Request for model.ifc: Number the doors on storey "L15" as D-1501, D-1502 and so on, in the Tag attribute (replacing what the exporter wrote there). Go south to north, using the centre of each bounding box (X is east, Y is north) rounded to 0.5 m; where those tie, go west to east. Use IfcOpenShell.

First a look at what the model holds.

```python
import ifcopenshell
import ifcopenshell.util.element
import ifcopenshell.util.placement

model = ifcopenshell.open("model.ifc")
print(model.schema)
storey = next(s for s in model.by_type("IfcBuildingStorey") if s.Name == "L15")
doors = [e for e in ifcopenshell.util.element.get_decomposition(storey) if e.is_a("IfcDoor")]
for e in sorted(doors, key=lambda e: e.id()):
    origin = ifcopenshell.util.placement.get_local_placement(e.ObjectPlacement)[:3, 3]
    print(e.id(), e.Tag, e.Name, origin.round(2) + 0.0, sep=" | ")
```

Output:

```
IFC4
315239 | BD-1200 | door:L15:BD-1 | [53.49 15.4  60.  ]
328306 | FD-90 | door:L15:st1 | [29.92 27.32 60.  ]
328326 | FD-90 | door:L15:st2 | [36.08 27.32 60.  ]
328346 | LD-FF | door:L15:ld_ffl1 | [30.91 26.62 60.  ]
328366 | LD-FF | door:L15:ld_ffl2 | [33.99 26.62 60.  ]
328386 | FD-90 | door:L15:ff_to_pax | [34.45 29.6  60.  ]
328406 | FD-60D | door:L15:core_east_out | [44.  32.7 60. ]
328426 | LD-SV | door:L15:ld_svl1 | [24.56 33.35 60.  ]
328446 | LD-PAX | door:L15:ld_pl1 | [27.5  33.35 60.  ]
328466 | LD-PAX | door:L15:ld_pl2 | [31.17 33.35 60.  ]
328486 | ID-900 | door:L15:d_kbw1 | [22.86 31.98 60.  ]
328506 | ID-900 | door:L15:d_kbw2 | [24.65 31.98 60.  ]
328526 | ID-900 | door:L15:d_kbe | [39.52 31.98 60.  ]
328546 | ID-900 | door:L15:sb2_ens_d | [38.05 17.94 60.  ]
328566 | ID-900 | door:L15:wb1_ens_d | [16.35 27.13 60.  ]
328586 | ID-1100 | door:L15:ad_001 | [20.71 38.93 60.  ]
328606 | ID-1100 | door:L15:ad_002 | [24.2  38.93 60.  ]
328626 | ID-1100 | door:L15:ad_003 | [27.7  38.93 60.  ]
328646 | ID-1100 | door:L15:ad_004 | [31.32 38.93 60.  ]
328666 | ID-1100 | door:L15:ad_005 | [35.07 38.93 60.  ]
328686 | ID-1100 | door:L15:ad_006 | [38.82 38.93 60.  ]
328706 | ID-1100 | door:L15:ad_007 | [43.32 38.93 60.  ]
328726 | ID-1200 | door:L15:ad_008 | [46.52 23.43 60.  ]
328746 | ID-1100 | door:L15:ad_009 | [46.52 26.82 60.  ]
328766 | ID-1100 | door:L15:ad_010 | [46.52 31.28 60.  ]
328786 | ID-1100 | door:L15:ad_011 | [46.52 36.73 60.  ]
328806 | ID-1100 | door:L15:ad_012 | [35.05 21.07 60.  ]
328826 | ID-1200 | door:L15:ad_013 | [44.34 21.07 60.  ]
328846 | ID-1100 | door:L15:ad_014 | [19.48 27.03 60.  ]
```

```python
import ifcopenshell
import ifcopenshell.geom
import ifcopenshell.util.element
import ifcopenshell.util.shape

model = ifcopenshell.open("model.ifc")
settings = ifcopenshell.geom.settings()
settings.set("use-world-coords", True)


def centre(element):
    shape = ifcopenshell.geom.create_shape(settings, element)
    return ifcopenshell.util.shape.get_bbox_centroid(shape.geometry)


storey = next(s for s in model.by_type("IfcBuildingStorey") if s.Name == "L15")
doors = [e for e in ifcopenshell.util.element.get_decomposition(storey) if e.is_a("IfcDoor")]

# Insertion points can sit at a corner or the storey origin, so sort by the geometry (in metres).
centres = {e: centre(e) for e in doors}
doors.sort(key=lambda e: (round(centres[e][1] / 0.5), centres[e][0]))

for i, e in enumerate(doors, start=1):
    number = f"D-15{i:02d}"
    e.Tag = number
    print(e.id(), number)

model.write("model_v2.ifc")
```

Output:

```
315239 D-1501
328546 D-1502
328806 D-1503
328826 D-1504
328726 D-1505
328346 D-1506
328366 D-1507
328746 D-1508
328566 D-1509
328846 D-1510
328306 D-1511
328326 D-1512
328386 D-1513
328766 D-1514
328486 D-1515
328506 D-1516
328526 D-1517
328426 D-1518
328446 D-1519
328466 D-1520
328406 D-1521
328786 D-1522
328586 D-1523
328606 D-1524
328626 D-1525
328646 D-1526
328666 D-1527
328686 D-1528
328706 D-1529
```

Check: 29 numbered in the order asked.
